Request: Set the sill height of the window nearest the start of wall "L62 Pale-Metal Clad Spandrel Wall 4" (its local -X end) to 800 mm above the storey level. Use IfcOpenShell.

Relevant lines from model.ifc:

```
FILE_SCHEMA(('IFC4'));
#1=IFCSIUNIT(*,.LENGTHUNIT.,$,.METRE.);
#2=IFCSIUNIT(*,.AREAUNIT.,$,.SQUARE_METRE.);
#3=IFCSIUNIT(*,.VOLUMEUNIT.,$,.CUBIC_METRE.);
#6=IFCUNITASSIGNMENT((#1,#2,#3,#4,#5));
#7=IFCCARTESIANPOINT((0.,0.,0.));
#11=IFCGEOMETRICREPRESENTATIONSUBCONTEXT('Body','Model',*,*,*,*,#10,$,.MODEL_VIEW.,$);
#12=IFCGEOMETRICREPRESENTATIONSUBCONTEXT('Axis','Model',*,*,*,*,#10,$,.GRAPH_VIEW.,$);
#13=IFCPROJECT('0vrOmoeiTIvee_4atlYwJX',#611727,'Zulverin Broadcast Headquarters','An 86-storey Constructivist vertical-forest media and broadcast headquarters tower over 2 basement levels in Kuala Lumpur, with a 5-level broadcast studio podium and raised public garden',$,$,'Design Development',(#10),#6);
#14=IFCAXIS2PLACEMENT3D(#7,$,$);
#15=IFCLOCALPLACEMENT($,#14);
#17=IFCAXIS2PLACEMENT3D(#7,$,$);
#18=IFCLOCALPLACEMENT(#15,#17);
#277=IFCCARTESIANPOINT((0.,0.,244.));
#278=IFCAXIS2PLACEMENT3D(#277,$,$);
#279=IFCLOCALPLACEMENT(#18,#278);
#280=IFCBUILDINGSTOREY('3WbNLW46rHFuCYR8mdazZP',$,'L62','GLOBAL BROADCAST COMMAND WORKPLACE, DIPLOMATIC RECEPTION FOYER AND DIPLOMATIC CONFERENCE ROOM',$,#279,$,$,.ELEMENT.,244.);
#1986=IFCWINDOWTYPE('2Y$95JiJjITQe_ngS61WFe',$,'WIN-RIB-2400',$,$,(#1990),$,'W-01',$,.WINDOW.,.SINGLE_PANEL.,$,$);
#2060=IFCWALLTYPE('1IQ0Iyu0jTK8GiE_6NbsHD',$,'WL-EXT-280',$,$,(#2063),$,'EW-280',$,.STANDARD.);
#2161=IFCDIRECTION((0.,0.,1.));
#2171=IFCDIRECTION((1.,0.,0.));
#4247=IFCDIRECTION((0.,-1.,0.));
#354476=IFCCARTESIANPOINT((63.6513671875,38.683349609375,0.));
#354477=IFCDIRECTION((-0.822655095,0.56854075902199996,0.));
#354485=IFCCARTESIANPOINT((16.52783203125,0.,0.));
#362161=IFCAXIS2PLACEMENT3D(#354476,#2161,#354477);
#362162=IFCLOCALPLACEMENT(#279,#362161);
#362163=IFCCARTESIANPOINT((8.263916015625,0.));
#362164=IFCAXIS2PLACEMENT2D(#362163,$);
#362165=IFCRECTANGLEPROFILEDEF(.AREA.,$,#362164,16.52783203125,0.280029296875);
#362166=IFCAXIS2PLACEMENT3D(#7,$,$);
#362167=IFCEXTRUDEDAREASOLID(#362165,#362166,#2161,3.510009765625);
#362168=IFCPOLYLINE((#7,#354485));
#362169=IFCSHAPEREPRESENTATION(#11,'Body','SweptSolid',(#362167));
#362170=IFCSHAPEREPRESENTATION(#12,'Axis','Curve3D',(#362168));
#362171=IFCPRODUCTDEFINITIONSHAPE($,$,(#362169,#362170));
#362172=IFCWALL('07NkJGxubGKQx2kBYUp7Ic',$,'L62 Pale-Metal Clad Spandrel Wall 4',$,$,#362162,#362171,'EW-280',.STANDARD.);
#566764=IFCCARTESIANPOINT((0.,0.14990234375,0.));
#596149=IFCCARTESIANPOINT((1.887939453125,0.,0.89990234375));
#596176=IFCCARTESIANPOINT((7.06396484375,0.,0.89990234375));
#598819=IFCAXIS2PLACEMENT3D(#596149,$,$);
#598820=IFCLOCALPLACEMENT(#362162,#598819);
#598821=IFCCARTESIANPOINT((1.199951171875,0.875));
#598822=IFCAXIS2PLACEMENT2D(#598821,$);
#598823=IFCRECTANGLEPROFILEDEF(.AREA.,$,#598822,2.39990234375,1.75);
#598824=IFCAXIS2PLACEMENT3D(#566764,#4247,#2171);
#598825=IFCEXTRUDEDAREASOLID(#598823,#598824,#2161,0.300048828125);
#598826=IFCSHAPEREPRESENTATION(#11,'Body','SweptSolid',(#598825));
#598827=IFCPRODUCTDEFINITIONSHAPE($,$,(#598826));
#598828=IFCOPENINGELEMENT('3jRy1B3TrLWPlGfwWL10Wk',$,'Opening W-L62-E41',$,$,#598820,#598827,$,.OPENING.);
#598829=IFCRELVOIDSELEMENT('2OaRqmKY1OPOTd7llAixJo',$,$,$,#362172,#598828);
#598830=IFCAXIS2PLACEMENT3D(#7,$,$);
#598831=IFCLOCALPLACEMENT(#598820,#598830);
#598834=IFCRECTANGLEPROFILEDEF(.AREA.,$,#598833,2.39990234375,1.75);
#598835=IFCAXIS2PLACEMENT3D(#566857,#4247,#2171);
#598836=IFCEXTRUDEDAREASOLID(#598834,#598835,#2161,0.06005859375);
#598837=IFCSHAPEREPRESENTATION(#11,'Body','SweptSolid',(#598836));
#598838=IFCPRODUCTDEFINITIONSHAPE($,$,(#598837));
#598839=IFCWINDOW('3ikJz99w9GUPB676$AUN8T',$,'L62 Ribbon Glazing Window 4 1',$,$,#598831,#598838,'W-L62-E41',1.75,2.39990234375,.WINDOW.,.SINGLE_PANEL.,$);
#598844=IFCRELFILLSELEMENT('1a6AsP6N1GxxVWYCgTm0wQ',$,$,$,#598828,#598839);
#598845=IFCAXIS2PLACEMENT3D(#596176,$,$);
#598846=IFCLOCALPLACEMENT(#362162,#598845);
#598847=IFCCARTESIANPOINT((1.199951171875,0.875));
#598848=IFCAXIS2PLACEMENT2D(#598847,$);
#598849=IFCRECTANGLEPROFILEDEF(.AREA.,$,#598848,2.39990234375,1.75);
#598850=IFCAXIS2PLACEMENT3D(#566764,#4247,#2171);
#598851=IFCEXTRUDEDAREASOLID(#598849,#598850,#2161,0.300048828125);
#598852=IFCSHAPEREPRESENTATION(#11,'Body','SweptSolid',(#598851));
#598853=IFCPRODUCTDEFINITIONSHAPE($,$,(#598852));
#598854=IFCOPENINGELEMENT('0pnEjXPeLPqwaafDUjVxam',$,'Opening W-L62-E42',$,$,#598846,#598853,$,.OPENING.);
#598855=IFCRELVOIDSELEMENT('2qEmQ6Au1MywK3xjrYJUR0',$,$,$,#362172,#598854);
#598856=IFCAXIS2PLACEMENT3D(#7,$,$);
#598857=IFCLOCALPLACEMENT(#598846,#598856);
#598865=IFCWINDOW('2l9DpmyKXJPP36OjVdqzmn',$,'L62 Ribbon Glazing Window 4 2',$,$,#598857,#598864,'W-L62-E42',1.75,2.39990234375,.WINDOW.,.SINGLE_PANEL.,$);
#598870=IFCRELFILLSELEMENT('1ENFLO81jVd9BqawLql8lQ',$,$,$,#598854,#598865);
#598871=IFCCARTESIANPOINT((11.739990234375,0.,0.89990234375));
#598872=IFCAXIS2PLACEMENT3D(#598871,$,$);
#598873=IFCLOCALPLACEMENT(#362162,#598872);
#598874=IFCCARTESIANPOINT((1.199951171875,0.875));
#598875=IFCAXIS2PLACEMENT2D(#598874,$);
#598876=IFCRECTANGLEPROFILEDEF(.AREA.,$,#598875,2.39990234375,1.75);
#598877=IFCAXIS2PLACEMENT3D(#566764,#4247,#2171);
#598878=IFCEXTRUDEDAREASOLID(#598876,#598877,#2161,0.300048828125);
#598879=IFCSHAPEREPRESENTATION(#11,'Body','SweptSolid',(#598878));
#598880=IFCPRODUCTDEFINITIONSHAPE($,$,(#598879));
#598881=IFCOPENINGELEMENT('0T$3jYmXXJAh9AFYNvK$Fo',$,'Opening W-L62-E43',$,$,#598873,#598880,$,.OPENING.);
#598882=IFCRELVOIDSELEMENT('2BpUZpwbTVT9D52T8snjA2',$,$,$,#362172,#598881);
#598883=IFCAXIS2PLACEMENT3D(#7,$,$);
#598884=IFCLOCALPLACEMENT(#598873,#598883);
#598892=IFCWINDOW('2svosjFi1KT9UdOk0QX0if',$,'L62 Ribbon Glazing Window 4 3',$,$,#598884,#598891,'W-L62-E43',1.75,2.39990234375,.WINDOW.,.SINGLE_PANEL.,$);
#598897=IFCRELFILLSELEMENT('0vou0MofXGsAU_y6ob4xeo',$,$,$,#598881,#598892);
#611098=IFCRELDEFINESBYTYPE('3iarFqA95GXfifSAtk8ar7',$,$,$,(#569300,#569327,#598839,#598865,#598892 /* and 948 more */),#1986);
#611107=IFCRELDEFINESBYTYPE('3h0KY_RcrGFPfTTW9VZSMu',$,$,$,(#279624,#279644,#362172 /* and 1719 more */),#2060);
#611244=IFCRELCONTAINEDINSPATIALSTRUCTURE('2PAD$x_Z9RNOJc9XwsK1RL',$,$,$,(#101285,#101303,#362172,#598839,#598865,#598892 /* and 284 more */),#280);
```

```python
import numpy as np
import ifcopenshell
import ifcopenshell.api.geometry
import ifcopenshell.geom
import ifcopenshell.util.element
import ifcopenshell.util.placement
import ifcopenshell.util.shape
import ifcopenshell.util.unit

model = ifcopenshell.open("model.ifc")
unit_scale = ifcopenshell.util.unit.calculate_unit_scale(model)

window = model.by_guid("3ikJz99w9GUPB676$AUN8T")
opening = window.FillsVoids[0].RelatingOpeningElement
storey = ifcopenshell.util.element.get_container(window, ifc_class="IfcBuildingStorey")
level = ifcopenshell.util.placement.get_local_placement(storey.ObjectPlacement)[2, 3]

# The opening's origin need not be at the sill, so measure its lowest point.
shape = ifcopenshell.geom.create_shape(ifcopenshell.geom.settings(), opening)
bottom = ifcopenshell.util.shape.get_shape_bottom_elevation(shape, shape.geometry) / unit_scale
dz = level + 0.8 / unit_scale - bottom

shift = np.array([0.0, 0.0, dz])
# The window is placed relative to its opening, so it follows when the opening moves.
matrix = ifcopenshell.util.placement.get_local_placement(opening.ObjectPlacement)
matrix[:3, 3] += shift
ifcopenshell.api.geometry.edit_object_placement(
    model, product=opening, matrix=matrix, is_si=False, should_transform_children=True
)

print(f"moved by {dz * unit_scale:+.3f} m")

model.write("model_v2.ifc")
```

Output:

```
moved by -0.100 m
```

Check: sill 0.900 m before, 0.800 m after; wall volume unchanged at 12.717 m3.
